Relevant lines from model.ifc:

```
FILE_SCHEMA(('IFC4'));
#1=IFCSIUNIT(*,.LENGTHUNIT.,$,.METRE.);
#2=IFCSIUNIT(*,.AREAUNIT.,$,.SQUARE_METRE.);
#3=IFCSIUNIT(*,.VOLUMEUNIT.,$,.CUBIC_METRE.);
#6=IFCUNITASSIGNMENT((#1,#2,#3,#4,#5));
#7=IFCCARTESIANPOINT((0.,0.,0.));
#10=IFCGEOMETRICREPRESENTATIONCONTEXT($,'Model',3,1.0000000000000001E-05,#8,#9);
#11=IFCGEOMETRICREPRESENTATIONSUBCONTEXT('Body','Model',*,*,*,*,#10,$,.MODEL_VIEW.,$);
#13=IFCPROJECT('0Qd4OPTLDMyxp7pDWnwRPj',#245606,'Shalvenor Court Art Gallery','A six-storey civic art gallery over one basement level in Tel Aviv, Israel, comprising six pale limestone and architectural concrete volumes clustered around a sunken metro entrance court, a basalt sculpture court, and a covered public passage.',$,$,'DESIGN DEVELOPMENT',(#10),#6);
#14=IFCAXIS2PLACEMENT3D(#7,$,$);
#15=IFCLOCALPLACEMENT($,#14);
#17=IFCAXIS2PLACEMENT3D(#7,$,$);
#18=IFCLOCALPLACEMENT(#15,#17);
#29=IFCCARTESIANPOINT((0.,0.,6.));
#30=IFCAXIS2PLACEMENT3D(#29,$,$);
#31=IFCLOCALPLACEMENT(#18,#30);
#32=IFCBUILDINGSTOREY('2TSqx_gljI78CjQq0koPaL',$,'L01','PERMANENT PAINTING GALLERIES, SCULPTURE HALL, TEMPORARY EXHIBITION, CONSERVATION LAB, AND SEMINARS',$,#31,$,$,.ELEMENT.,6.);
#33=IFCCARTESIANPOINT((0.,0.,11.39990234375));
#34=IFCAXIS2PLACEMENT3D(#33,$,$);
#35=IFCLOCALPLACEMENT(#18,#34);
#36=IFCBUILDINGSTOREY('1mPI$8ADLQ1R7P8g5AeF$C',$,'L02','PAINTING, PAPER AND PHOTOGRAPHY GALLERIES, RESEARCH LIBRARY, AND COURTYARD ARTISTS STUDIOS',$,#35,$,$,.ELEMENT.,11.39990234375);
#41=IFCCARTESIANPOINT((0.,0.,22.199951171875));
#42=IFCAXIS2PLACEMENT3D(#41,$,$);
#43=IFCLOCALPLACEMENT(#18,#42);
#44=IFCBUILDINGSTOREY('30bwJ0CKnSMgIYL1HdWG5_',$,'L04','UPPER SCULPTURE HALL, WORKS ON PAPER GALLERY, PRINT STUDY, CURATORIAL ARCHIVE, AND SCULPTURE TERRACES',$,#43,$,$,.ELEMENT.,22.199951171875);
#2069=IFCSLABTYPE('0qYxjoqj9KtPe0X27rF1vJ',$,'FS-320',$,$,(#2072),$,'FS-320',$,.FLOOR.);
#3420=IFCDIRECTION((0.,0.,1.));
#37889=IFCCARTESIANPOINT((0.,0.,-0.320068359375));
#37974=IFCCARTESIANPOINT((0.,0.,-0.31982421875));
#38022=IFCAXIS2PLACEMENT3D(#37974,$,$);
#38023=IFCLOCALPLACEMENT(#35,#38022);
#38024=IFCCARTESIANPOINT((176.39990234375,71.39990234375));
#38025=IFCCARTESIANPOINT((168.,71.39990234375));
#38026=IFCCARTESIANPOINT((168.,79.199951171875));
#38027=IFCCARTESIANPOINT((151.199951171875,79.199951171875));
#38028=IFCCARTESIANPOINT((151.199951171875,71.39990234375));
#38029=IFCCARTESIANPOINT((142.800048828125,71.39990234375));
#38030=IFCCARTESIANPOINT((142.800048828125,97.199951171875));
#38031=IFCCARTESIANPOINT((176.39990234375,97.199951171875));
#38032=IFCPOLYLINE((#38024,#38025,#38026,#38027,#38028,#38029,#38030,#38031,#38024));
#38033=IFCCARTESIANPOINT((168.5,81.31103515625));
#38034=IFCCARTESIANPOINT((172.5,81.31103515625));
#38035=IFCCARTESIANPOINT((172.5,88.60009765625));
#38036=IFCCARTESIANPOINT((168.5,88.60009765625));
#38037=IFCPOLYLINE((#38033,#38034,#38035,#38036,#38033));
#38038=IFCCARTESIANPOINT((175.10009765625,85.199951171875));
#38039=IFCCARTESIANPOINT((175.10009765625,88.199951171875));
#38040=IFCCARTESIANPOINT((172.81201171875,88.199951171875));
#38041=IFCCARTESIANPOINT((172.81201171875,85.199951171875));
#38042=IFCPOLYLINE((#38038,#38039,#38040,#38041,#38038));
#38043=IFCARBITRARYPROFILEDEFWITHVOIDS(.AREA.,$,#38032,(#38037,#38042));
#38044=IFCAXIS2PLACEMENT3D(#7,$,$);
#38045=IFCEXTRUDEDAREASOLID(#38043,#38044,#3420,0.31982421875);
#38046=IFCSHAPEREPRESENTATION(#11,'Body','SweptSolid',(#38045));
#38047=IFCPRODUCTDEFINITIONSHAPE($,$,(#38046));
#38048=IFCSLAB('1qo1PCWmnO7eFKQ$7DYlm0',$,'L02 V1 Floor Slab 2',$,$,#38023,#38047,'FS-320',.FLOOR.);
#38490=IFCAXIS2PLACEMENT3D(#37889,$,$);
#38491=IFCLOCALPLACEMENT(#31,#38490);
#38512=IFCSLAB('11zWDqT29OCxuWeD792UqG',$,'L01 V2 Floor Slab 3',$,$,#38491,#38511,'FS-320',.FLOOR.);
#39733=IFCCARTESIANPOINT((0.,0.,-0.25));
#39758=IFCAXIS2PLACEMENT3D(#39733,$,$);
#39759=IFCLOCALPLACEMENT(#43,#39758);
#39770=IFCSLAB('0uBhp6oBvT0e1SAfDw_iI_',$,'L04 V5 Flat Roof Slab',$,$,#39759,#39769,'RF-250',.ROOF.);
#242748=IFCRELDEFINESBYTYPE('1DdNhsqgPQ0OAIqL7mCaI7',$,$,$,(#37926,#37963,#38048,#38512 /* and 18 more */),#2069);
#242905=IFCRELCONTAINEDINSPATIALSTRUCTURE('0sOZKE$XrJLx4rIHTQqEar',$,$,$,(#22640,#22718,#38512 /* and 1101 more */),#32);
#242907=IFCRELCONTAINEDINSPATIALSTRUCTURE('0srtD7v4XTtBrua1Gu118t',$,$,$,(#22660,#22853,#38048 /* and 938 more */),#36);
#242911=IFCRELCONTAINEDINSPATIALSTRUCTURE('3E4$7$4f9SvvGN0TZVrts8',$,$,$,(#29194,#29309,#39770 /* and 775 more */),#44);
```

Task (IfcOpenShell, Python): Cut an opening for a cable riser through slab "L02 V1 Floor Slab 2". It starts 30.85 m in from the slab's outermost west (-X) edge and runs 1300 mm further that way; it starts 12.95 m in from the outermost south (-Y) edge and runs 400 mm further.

```python
import numpy as np
import ifcopenshell
import ifcopenshell.api.feature
import ifcopenshell.api.geometry
import ifcopenshell.api.root
import ifcopenshell.geom
import ifcopenshell.util.placement
import ifcopenshell.util.representation
import ifcopenshell.util.shape
import ifcopenshell.util.unit

model = ifcopenshell.open("model.ifc")
unit_scale = ifcopenshell.util.unit.calculate_unit_scale(model)
settings = ifcopenshell.geom.settings()


def volume(element):
    """Net volume in cubic metres, openings subtracted."""
    shape = ifcopenshell.geom.create_shape(settings, element)
    return ifcopenshell.util.shape.get_volume(shape.geometry)


slab = model.by_id(38048)
before = volume(slab)

# Extent in the slab's own axes, in metres. The edges named are its -X and -Y sides.
slab_shape = ifcopenshell.geom.create_shape(settings, slab)
vertices = ifcopenshell.util.shape.get_vertices(slab_shape.geometry)
x_min, y_min, bottom = vertices.min(axis=0)
top = vertices[:, 2].max()

opening = ifcopenshell.api.root.create_entity(model, ifc_class="IfcOpeningElement", name="Cable riser opening", predefined_type="OPENING")
context = ifcopenshell.util.representation.get_context(model, "Model", "Body", "MODEL_VIEW")
width, depth = 1.3, 0.4
outline = [(0.0, 0.0), (width, 0.0), (width, depth), (0.0, depth), (0.0, 0.0)]
# Overshoot both faces by 50 mm so the cut is clean.
shape = ifcopenshell.api.geometry.add_slab_representation(
    model, context=context, depth=top - bottom + 0.1, polyline=outline
)
ifcopenshell.api.geometry.assign_representation(model, product=opening, representation=shape)

matrix = ifcopenshell.util.placement.get_local_placement(slab.ObjectPlacement)
matrix[:, 3] = matrix @ np.append(np.array([x_min + 30.85, y_min + 12.95, bottom - 0.05]) / unit_scale, 1.0)
ifcopenshell.api.geometry.edit_object_placement(model, product=opening, matrix=matrix, is_si=False)
ifcopenshell.api.feature.add_feature(model, feature=opening, element=slab)

after = volume(slab)

print(f"slab volume {before:.3f} -> {after:.3f} m3")

model.write("model-out.ifc")
```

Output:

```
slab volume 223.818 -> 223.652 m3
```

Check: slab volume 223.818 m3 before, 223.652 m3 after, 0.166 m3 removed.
